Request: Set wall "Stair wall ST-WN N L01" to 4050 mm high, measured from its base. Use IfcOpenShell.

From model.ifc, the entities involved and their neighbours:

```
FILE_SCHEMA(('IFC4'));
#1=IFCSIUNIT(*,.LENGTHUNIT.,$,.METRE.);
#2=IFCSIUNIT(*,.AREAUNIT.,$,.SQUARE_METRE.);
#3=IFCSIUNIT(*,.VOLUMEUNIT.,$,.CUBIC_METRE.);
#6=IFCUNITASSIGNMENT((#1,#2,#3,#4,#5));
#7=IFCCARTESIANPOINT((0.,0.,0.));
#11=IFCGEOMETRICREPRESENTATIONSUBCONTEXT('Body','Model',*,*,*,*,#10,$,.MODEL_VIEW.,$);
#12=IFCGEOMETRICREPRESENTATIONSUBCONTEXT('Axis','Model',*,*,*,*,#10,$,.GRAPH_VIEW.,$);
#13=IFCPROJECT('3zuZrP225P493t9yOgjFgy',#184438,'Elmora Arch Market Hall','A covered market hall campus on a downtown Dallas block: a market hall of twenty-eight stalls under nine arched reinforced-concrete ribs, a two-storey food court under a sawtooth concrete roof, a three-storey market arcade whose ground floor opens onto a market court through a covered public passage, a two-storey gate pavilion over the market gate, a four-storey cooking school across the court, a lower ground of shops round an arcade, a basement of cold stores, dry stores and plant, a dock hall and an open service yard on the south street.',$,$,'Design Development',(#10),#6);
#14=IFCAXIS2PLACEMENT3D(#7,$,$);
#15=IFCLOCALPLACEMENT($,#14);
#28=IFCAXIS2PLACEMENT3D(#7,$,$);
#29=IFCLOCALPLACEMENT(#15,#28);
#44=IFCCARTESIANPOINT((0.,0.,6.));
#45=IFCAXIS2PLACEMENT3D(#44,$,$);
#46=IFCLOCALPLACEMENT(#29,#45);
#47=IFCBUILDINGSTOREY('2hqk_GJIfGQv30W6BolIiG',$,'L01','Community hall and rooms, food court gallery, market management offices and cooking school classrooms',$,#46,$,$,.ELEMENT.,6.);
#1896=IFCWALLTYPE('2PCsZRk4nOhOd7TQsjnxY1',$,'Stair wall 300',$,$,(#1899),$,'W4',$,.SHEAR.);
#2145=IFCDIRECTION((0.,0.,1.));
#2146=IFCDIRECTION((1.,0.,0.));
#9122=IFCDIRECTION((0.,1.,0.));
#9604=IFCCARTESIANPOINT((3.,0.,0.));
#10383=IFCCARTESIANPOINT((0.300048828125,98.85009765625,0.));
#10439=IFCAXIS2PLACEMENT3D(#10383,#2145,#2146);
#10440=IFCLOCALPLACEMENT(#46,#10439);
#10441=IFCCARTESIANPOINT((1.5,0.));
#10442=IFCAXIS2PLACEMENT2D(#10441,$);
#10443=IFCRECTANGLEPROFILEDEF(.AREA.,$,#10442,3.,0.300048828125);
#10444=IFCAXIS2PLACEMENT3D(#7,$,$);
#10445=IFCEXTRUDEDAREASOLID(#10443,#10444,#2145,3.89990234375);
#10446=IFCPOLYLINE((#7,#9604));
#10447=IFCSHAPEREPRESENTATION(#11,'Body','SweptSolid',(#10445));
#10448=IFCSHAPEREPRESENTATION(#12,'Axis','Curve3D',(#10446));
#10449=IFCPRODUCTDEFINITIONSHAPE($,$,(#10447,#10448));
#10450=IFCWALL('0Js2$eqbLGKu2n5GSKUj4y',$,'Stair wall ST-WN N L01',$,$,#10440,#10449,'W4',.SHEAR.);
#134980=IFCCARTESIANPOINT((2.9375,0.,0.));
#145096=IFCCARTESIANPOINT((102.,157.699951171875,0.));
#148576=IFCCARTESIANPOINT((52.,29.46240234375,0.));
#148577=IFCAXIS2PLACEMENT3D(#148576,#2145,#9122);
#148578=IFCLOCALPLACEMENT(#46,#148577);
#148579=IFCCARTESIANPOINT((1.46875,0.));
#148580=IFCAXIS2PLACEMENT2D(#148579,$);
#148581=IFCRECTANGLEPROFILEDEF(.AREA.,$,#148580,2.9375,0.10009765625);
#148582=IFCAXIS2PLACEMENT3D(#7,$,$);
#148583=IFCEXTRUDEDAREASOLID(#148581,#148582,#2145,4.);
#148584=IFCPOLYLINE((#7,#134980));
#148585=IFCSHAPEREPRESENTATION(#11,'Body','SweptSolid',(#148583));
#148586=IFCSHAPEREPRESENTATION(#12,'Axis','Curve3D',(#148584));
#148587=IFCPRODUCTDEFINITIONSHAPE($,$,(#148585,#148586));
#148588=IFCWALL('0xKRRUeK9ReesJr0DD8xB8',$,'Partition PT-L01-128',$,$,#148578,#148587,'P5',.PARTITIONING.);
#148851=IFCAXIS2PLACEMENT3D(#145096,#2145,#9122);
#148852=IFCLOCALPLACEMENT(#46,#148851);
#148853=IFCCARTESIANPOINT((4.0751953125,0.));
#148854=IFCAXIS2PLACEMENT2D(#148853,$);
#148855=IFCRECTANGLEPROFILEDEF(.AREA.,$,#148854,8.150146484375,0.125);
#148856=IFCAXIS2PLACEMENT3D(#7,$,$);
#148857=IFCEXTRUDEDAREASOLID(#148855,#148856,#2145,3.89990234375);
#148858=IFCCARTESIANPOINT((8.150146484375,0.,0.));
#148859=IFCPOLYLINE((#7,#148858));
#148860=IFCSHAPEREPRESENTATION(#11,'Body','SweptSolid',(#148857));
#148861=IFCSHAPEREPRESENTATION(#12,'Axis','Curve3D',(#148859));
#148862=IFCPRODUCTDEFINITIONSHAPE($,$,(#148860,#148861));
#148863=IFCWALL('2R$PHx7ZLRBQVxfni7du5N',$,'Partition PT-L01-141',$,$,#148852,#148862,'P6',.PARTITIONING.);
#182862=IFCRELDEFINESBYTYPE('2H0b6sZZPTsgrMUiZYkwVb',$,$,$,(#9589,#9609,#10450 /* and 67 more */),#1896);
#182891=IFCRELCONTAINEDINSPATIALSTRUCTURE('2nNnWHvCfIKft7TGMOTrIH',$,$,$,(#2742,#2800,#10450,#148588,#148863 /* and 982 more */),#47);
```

```python
import ifcopenshell
import ifcopenshell.geom
import ifcopenshell.util.representation
import ifcopenshell.util.shape

model = ifcopenshell.open("model.ifc")
settings = ifcopenshell.geom.settings()


def volume(element):
    """Net volume in cubic metres, openings subtracted."""
    shape = ifcopenshell.geom.create_shape(settings, element)
    return ifcopenshell.util.shape.get_volume(shape.geometry)


wall = model.by_guid("0Js2$eqbLGKu2n5GSKUj4y")
before = volume(wall)

body = ifcopenshell.util.representation.get_representation(wall, "Model", "Body")
solid = body.Items[0]
old_height = solid.Depth
solid.Depth = 4.05
after = volume(wall)

print(f"height {old_height:g} -> {solid.Depth:g}, volume {before:.3f} -> {after:.3f} m3")

model.write("model_updated.ifc")
```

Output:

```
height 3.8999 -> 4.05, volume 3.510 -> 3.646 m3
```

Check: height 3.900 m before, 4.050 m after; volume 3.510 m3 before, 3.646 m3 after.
